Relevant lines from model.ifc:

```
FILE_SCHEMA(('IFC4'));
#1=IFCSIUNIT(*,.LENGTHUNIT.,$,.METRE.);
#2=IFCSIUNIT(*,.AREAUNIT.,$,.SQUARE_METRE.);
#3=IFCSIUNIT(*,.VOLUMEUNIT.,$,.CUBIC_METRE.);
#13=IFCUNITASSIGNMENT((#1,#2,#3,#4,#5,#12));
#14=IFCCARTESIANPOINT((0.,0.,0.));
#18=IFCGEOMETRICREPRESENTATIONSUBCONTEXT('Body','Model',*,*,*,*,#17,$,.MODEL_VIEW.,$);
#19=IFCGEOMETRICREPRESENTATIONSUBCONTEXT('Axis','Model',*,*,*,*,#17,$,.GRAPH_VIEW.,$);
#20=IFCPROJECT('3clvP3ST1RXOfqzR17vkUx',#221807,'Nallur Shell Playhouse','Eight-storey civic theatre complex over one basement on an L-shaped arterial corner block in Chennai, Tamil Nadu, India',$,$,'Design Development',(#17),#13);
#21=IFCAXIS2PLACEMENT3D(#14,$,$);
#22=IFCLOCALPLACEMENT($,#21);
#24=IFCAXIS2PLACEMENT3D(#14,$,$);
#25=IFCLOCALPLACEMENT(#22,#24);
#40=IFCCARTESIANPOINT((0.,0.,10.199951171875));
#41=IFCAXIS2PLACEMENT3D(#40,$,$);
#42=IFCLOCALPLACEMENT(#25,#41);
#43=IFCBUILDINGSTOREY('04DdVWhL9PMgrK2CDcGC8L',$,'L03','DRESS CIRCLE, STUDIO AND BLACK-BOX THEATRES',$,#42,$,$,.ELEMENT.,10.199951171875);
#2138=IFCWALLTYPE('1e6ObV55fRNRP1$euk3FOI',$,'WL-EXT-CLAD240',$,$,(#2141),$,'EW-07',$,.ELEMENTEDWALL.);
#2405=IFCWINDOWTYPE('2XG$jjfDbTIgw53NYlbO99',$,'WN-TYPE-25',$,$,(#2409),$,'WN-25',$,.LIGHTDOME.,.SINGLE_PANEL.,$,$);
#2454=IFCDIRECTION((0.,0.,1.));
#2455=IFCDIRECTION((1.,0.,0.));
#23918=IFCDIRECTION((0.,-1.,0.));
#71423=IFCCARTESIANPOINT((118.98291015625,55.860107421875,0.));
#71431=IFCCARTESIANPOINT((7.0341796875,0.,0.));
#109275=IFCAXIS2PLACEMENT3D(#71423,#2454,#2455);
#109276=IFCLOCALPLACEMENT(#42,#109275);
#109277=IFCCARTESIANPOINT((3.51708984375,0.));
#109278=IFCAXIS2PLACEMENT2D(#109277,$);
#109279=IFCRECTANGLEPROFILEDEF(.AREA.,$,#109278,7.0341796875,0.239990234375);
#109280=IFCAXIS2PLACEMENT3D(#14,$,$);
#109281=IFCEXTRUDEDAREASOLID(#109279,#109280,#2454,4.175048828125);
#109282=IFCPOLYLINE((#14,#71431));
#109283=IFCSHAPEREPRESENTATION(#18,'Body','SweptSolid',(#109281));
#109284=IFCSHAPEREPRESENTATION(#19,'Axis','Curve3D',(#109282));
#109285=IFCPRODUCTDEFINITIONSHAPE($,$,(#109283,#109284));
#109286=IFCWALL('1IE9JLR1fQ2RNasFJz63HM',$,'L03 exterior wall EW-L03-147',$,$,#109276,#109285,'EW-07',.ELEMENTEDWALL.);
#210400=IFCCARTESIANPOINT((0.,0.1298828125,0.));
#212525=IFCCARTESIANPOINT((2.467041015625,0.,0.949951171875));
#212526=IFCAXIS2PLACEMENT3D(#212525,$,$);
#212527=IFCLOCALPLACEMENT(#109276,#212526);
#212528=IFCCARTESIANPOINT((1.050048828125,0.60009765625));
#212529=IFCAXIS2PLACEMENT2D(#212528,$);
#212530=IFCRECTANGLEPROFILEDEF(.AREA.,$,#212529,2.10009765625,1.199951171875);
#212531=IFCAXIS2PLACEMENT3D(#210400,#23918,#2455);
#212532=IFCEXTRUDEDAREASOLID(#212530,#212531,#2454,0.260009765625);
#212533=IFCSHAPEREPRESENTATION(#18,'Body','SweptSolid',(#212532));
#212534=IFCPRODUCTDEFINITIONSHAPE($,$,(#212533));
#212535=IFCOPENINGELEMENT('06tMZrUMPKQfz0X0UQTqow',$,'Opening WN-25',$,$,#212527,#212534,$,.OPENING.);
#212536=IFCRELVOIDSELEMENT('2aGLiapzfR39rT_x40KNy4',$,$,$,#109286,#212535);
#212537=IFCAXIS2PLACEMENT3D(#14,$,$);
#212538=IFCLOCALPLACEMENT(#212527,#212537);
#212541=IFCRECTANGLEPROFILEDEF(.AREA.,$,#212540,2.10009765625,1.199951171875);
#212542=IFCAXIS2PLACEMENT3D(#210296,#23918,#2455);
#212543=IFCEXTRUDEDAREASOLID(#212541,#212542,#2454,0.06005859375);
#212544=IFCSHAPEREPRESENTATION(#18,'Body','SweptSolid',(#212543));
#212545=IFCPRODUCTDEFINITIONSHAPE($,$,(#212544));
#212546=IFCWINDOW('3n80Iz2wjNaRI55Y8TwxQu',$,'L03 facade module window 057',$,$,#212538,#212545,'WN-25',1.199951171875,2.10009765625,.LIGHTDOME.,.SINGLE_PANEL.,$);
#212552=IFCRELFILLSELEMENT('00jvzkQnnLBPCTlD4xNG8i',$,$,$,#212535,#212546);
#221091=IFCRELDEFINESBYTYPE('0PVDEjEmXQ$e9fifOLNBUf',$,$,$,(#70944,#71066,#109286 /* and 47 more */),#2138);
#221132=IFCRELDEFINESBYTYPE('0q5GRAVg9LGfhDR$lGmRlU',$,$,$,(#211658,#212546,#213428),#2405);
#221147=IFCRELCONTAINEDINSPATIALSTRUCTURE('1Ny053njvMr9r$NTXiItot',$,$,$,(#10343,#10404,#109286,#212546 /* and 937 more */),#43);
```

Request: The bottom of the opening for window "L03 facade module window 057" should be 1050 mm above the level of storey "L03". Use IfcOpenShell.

```python
import numpy as np
import ifcopenshell
import ifcopenshell.api.geometry
import ifcopenshell.geom
import ifcopenshell.util.element
import ifcopenshell.util.placement
import ifcopenshell.util.shape
import ifcopenshell.util.unit

model = ifcopenshell.open("model.ifc")
unit_scale = ifcopenshell.util.unit.calculate_unit_scale(model)

window = model.by_id(212546)
opening = window.FillsVoids[0].RelatingOpeningElement
storey = ifcopenshell.util.element.get_container(window, ifc_class="IfcBuildingStorey")
level = ifcopenshell.util.placement.get_local_placement(storey.ObjectPlacement)[2, 3]

# The opening's origin need not be at the sill, so measure its lowest point.
shape = ifcopenshell.geom.create_shape(ifcopenshell.geom.settings(), opening)
bottom = ifcopenshell.util.shape.get_shape_bottom_elevation(shape, shape.geometry) / unit_scale
dz = level + 1.05 - bottom

shift = np.array([0.0, 0.0, dz])
# The window is placed relative to its opening, so it follows when the opening moves.
matrix = ifcopenshell.util.placement.get_local_placement(opening.ObjectPlacement)
matrix[:3, 3] += shift
ifcopenshell.api.geometry.edit_object_placement(
    model, product=opening, matrix=matrix, is_si=False, should_transform_children=True
)

print(f"moved by {dz * unit_scale:+.3f} m")

model.write("model_rev.ifc")
```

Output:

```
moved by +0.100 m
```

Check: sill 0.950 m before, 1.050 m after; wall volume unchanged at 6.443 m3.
